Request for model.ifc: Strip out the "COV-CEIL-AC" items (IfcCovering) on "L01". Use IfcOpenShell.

First a look at what the model holds.

```python
import ifcopenshell
import ifcopenshell.util.element

model = ifcopenshell.open("model.ifc")
print(model.schema)
storey = next(s for s in model.by_type("IfcBuildingStorey") if s.Name == "L01")
coverings = [e for e in ifcopenshell.util.element.get_decomposition(storey) if e.is_a("IfcCovering")]
seen = {}
for e in coverings:
    element_type = ifcopenshell.util.element.get_type(e)
    name = element_type.Name if element_type not in (None, e) else None
    seen[name] = seen.get(name, 0) + 1
for name, count in sorted(seen.items(), key=str):
    print(count, "x", name)
```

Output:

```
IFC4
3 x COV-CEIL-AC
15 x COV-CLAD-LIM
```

```python
import ifcopenshell
import ifcopenshell.api.root
import ifcopenshell.util.element

model = ifcopenshell.open("model.ifc")

storey = next(s for s in model.by_type("IfcBuildingStorey") if s.Name == "L01")
coverings = [e for e in ifcopenshell.util.element.get_decomposition(storey) if e.is_a("IfcCovering")]
targets = [e for e in coverings if (t := ifcopenshell.util.element.get_type(e)) not in (None, e) and t.Name == "COV-CEIL-AC"]

for e in targets:
    ifcopenshell.api.root.remove_product(model, product=e)
print(len(targets), "removed")

model.write("model-out.ifc")
```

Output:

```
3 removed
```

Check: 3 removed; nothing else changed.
